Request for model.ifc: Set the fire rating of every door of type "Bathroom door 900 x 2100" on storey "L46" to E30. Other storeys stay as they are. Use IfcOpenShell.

First a look at what the model holds.

```python
import ifcopenshell
import ifcopenshell.util.element

model = ifcopenshell.open("model.ifc")
print(model.schema)
storey = next(s for s in model.by_type("IfcBuildingStorey") if s.Name == "L46")
doors = [e for e in ifcopenshell.util.element.get_decomposition(storey) if e.is_a("IfcDoor")]
seen = {}
for e in doors:
    element_type = ifcopenshell.util.element.get_type(e)
    key = (element_type.Name if element_type != e and element_type else None, ifcopenshell.util.element.get_pset(e, "Pset_DoorCommon", "FireRating"))
    seen[key] = seen.get(key, 0) + 1
for (name, value), count in sorted(seen.items(), key=str):
    print(count, "x", name, "|", value)
```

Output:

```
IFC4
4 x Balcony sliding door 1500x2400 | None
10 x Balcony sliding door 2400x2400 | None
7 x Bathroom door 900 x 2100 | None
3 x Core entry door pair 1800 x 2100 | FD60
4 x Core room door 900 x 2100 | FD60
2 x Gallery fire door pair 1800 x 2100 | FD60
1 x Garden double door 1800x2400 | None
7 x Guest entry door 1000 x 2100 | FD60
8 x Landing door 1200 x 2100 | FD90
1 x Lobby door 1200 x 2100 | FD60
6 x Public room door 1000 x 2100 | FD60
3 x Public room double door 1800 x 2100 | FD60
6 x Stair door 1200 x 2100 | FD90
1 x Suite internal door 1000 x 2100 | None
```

```python
import ifcopenshell
import ifcopenshell.api.pset
import ifcopenshell.util.element

model = ifcopenshell.open("model.ifc")

storey = next(s for s in model.by_type("IfcBuildingStorey") if s.Name == "L46")
doors = [e for e in ifcopenshell.util.element.get_decomposition(storey) if e.is_a("IfcDoor")]

count = 0
for e in doors:
    element_type = ifcopenshell.util.element.get_type(e)
    if element_type in (None, e) or element_type.Name != "Bathroom door 900 x 2100":
        continue
    # add_pset returns the element's existing set when there is one.
    pset = ifcopenshell.api.pset.add_pset(model, product=e, name="Pset_DoorCommon")
    ifcopenshell.api.pset.edit_pset(model, pset=pset, properties={"FireRating": "E30"})
    count += 1

print(count, "doors updated")

model.write("model_updated.ifc")
```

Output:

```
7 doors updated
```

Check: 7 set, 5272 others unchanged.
